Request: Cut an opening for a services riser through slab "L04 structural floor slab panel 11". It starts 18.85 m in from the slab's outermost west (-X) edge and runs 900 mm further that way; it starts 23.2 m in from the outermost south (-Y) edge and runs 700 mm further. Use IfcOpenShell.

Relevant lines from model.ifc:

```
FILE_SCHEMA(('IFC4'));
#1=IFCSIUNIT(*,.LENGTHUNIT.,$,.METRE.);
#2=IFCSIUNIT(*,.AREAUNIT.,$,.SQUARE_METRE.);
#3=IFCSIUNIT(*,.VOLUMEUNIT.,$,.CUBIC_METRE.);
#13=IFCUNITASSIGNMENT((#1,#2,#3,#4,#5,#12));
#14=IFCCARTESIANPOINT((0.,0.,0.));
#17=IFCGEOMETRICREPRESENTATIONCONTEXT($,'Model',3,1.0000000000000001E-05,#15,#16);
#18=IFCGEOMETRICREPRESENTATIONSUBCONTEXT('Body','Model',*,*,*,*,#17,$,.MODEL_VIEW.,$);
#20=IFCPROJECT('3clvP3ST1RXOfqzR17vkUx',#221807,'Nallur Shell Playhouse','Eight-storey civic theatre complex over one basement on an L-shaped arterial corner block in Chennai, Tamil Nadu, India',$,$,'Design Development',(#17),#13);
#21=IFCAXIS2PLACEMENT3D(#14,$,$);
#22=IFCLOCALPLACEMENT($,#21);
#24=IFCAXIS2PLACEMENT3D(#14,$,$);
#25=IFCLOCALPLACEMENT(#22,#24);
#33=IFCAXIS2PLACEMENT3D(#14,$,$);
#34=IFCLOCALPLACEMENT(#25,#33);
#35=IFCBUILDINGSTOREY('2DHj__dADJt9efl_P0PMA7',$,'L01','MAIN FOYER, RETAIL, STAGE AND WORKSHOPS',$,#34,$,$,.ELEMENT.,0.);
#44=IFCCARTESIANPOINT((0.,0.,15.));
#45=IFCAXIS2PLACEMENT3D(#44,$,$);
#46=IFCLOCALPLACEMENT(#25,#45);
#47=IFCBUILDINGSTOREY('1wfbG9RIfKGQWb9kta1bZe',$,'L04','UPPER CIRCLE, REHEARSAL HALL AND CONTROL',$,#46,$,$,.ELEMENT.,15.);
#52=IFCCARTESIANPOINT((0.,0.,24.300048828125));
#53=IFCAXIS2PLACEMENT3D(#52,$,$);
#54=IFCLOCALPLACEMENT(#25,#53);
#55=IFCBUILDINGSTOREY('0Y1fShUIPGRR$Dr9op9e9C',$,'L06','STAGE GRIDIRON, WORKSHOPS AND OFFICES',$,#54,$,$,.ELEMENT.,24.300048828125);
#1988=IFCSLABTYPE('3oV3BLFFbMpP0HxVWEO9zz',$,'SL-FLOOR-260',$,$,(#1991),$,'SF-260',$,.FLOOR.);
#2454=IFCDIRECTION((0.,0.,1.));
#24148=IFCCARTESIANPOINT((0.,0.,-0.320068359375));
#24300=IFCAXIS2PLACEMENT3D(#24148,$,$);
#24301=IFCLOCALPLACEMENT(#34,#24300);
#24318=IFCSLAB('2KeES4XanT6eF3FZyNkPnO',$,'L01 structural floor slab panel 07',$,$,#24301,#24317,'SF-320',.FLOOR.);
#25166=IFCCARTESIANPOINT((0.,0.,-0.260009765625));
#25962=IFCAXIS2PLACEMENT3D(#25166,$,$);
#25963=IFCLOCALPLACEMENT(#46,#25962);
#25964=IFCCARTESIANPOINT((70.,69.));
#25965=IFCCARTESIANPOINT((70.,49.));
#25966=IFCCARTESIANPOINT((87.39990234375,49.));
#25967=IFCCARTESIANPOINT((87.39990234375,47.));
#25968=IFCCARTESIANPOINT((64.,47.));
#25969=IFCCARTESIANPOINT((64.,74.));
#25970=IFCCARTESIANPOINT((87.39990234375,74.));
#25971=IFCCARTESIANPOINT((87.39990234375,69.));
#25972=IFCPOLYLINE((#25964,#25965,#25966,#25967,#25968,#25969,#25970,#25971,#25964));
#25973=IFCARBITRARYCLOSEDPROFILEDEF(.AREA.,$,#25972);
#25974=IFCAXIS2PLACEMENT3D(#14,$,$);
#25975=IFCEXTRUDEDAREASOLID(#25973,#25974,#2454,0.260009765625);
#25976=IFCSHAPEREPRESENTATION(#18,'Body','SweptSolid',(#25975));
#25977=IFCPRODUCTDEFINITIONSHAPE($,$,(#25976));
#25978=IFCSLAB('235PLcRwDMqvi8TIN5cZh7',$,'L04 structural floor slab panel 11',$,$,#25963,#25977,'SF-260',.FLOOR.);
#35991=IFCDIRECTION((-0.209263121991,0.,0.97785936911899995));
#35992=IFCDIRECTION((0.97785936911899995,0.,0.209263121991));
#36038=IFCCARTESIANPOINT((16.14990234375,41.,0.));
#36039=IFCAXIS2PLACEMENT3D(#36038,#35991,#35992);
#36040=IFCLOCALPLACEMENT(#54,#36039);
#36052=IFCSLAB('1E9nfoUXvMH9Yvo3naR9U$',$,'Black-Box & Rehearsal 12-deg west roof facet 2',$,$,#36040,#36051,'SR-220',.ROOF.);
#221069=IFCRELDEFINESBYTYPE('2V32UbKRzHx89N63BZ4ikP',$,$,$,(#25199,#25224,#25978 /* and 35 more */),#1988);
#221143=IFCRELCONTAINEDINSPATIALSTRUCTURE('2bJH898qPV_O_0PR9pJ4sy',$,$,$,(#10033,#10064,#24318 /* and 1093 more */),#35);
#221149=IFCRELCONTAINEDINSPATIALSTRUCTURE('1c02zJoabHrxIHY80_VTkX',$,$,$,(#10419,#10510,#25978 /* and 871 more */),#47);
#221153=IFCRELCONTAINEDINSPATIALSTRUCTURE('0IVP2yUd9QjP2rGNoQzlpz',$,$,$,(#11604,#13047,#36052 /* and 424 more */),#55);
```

```python
import numpy as np
import ifcopenshell
import ifcopenshell.api.feature
import ifcopenshell.api.geometry
import ifcopenshell.api.root
import ifcopenshell.geom
import ifcopenshell.util.placement
import ifcopenshell.util.representation
import ifcopenshell.util.shape
import ifcopenshell.util.unit

model = ifcopenshell.open("model.ifc")
unit_scale = ifcopenshell.util.unit.calculate_unit_scale(model)
settings = ifcopenshell.geom.settings()


def volume(element):
    """Net volume in cubic metres, openings subtracted."""
    shape = ifcopenshell.geom.create_shape(settings, element)
    return ifcopenshell.util.shape.get_volume(shape.geometry)


slab = model.by_guid("235PLcRwDMqvi8TIN5cZh7")
before = volume(slab)

# Extent in the slab's own axes, in metres. The edges named are its -X and -Y sides.
slab_shape = ifcopenshell.geom.create_shape(settings, slab)
vertices = ifcopenshell.util.shape.get_vertices(slab_shape.geometry)
x_min, y_min, bottom = vertices.min(axis=0)
top = vertices[:, 2].max()

opening = ifcopenshell.api.root.create_entity(model, ifc_class="IfcOpeningElement", name="Services riser opening", predefined_type="OPENING")
context = ifcopenshell.util.representation.get_context(model, "Model", "Body", "MODEL_VIEW")
width, depth = 0.9, 0.7
outline = [(0.0, 0.0), (width, 0.0), (width, depth), (0.0, depth), (0.0, 0.0)]
# Overshoot both faces by 50 mm so the cut is clean.
shape = ifcopenshell.api.geometry.add_slab_representation(
    model, context=context, depth=top - bottom + 0.1, polyline=outline
)
ifcopenshell.api.geometry.assign_representation(model, product=opening, representation=shape)

matrix = ifcopenshell.util.placement.get_local_placement(slab.ObjectPlacement)
matrix[:, 3] = matrix @ np.append(np.array([x_min + 18.85, y_min + 23.2, bottom - 0.05]) / unit_scale, 1.0)
ifcopenshell.api.geometry.edit_object_placement(model, product=opening, matrix=matrix, is_si=False)
ifcopenshell.api.feature.add_feature(model, feature=opening, element=slab)

after = volume(slab)

print(f"slab volume {before:.3f} -> {after:.3f} m3")

model.write("model_v2.ifc")
```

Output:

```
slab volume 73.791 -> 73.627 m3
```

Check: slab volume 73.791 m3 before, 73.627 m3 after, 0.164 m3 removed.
